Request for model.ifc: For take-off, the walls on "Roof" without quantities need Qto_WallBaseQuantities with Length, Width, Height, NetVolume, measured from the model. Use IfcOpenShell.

First a look at what the model holds.

```python
import ifcopenshell
import ifcopenshell.util.element
import ifcopenshell.util.unit

model = ifcopenshell.open("model.ifc")
print(model.schema)
for unit_type in ("LENGTHUNIT", "AREAUNIT", "VOLUMEUNIT"):
    print(unit_type, ifcopenshell.util.unit.calculate_unit_scale(model, unit_type))
storey = next(s for s in model.by_type("IfcBuildingStorey") if s.Name == "Roof")
walls = [e for e in ifcopenshell.util.element.get_decomposition(storey) if e.is_a("IfcWall")]
for e in sorted(walls, key=lambda e: e.id()):
    print(e.id(), e.is_a(), e.Name, list(ifcopenshell.util.element.get_psets(e, qtos_only=True)), sep=" | ")
```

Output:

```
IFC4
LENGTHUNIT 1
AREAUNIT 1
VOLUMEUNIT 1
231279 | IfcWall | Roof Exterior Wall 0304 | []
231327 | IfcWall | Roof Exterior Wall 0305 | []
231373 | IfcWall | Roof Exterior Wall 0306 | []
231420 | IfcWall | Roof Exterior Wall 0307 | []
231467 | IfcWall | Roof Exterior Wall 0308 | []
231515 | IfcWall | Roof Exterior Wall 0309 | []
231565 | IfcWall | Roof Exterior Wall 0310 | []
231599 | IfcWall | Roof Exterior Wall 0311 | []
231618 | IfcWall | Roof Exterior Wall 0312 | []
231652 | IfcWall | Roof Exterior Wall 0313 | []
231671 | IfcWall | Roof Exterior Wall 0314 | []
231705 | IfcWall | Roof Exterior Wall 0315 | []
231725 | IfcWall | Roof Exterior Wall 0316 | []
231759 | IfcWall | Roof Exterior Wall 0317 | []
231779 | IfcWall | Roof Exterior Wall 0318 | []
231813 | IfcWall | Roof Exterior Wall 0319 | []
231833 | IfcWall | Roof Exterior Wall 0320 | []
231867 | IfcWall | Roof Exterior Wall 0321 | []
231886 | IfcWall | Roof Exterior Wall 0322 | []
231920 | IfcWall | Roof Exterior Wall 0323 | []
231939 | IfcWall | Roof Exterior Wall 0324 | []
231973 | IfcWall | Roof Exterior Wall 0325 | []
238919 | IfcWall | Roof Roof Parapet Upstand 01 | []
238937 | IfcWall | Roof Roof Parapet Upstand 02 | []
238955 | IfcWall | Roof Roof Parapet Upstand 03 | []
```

```python
import ifcopenshell
import ifcopenshell.api.pset
import ifcopenshell.geom
import ifcopenshell.util.element
import ifcopenshell.util.shape
import ifcopenshell.util.unit

model = ifcopenshell.open("model.ifc")
unit_scale = ifcopenshell.util.unit.calculate_unit_scale(model)
volume_scale = ifcopenshell.util.unit.calculate_unit_scale(model, "VOLUMEUNIT")
settings = ifcopenshell.geom.settings()

storey = next(s for s in model.by_type("IfcBuildingStorey") if s.Name == "Roof")
walls = [e for e in ifcopenshell.util.element.get_decomposition(storey) if e.is_a("IfcWall")]

for e in sorted(walls, key=lambda e: e.id()):
    if ifcopenshell.util.element.get_psets(e, qtos_only=True, should_inherit=False):
        continue
    # Geometry comes back in metres, in the element's own axes.
    shape = ifcopenshell.geom.create_shape(settings, e)
    values = {
        "Length": ifcopenshell.util.shape.get_x(shape.geometry) / unit_scale,
        "Width": ifcopenshell.util.shape.get_y(shape.geometry) / unit_scale,
        "Height": ifcopenshell.util.shape.get_z(shape.geometry) / unit_scale,
        "NetVolume": ifcopenshell.util.shape.get_volume(shape.geometry) / volume_scale,
    }
    qto = ifcopenshell.api.pset.add_qto(model, product=e, name="Qto_WallBaseQuantities")
    ifcopenshell.api.pset.edit_qto(model, qto=qto, properties=values)
    print(e.id(), {k: round(v, 3) for k, v in values.items()})

model.write("model_rev.ifc")
```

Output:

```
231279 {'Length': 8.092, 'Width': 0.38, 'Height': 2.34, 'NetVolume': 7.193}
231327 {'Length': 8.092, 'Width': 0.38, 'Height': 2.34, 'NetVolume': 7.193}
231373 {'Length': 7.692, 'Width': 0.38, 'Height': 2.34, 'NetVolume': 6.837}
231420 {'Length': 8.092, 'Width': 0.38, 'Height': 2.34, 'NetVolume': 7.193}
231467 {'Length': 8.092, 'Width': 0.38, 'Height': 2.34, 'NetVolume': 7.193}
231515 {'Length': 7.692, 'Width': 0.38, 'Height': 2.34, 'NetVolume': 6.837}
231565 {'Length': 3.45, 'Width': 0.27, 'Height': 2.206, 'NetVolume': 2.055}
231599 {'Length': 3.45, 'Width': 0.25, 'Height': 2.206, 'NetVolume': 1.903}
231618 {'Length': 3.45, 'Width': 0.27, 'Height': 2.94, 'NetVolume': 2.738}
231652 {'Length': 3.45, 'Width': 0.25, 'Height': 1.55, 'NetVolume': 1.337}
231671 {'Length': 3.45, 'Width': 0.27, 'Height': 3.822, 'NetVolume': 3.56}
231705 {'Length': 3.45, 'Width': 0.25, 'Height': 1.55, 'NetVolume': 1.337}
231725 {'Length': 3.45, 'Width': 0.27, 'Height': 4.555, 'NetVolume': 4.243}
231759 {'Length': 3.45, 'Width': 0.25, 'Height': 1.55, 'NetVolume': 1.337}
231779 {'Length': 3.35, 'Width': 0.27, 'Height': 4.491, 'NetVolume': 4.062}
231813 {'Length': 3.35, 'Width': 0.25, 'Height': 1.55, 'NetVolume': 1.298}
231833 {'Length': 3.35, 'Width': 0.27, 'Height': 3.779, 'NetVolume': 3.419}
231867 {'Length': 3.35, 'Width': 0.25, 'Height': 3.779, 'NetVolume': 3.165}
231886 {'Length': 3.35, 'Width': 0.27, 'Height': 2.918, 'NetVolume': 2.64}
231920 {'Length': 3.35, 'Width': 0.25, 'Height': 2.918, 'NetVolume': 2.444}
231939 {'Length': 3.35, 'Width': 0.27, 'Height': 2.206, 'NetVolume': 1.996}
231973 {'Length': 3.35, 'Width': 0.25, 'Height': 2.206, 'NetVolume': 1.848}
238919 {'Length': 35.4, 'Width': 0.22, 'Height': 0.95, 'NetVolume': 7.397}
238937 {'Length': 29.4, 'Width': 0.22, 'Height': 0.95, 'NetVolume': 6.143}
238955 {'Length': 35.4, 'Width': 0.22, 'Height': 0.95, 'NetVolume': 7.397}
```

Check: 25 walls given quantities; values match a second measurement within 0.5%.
